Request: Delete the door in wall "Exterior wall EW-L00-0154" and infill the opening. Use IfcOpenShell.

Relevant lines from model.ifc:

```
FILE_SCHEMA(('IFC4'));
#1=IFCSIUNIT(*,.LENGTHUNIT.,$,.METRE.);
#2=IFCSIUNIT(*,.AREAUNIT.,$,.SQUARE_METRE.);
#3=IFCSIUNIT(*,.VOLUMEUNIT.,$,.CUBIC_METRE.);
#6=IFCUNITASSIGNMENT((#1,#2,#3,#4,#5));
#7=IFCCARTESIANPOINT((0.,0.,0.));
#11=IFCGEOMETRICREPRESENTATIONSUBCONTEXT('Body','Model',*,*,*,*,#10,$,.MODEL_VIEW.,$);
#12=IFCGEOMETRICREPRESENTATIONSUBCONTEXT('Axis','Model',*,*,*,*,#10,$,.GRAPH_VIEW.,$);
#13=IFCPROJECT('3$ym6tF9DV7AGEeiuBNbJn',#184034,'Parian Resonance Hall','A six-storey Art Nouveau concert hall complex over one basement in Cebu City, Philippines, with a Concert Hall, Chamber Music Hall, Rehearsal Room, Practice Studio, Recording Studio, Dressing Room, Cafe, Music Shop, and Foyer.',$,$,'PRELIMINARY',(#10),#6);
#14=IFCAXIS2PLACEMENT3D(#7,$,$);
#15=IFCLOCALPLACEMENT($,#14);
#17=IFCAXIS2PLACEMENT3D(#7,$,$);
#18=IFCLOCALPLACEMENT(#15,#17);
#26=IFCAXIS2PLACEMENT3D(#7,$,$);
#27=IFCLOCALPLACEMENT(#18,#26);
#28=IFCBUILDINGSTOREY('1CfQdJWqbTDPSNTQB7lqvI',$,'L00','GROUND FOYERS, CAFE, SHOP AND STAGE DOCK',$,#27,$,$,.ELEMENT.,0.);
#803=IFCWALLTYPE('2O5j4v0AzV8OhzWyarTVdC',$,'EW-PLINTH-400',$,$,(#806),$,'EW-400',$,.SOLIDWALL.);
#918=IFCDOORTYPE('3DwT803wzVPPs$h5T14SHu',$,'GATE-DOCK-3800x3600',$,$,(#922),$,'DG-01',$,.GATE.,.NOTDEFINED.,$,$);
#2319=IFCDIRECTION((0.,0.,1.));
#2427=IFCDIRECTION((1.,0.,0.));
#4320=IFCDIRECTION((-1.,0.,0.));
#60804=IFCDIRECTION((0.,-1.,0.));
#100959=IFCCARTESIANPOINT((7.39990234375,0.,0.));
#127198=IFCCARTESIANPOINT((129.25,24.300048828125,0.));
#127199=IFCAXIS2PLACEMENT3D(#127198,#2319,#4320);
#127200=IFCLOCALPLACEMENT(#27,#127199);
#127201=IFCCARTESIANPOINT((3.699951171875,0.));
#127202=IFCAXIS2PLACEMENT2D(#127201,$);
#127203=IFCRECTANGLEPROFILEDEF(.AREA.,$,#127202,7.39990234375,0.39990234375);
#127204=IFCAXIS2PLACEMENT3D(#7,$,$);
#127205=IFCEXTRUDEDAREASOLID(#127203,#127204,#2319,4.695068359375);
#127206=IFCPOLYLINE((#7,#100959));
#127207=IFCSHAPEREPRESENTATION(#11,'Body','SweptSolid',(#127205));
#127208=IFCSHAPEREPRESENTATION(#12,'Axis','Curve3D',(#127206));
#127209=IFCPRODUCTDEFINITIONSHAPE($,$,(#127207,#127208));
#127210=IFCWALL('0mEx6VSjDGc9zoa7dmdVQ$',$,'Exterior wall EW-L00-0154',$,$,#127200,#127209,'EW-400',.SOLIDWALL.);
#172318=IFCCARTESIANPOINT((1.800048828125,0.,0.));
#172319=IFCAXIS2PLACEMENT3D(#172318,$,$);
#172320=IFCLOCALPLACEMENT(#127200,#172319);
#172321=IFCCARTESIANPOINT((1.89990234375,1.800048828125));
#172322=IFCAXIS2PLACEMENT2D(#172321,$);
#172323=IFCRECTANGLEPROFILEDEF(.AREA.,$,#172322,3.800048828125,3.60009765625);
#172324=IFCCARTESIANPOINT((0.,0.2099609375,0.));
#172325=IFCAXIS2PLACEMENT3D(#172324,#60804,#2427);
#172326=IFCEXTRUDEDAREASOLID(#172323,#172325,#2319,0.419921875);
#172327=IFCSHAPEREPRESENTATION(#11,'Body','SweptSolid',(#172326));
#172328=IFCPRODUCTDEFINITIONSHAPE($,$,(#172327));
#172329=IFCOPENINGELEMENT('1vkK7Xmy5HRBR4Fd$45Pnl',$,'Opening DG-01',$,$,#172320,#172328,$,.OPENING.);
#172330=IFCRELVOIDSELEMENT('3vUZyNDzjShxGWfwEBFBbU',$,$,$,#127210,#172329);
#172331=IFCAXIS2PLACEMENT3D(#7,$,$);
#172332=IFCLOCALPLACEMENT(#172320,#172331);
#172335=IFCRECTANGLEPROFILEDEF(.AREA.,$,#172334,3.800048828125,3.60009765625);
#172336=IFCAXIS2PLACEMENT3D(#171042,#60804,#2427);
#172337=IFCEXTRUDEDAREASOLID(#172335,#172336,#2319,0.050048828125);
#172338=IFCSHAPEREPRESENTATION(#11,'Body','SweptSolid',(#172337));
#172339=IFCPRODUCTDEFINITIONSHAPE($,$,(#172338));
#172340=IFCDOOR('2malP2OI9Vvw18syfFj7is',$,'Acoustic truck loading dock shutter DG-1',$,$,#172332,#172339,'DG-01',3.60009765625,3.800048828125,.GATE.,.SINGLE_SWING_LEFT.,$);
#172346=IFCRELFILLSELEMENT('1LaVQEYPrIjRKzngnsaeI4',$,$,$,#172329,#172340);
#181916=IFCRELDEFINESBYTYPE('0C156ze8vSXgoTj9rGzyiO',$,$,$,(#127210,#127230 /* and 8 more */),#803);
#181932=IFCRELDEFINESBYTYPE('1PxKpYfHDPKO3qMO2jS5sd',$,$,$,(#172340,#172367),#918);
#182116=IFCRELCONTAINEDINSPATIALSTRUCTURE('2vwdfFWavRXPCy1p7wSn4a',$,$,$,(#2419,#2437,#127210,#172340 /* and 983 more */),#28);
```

```python
import ifcopenshell
import ifcopenshell.api.feature
import ifcopenshell.api.root
import ifcopenshell.geom
import ifcopenshell.util.shape

model = ifcopenshell.open("model.ifc")
settings = ifcopenshell.geom.settings()


def volume(element):
    """Net volume in cubic metres, openings subtracted."""
    shape = ifcopenshell.geom.create_shape(settings, element)
    return ifcopenshell.util.shape.get_volume(shape.geometry)


door = model.by_id(172340)
opening = door.FillsVoids[0].RelatingOpeningElement
wall = opening.VoidsElements[0].RelatingBuildingElement
before = volume(wall)

ifcopenshell.api.root.remove_product(model, product=door)
ifcopenshell.api.feature.remove_feature(model, feature=opening)

after = volume(wall)

print(f"wall volume {before:.3f} -> {after:.3f} m3")

model.write("model_rev.ifc")
```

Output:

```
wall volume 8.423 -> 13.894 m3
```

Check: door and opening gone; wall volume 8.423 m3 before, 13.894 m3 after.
